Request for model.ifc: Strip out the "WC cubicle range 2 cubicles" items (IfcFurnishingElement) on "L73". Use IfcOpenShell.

First a look at what the model holds.

```python
import ifcopenshell
import ifcopenshell.util.element

model = ifcopenshell.open("model.ifc")
print(model.schema)
storey = next(s for s in model.by_type("IfcBuildingStorey") if s.Name == "L73")
furniture = [e for e in ifcopenshell.util.element.get_decomposition(storey) if e.is_a("IfcFurnishingElement")]
seen = {}
for e in furniture:
    element_type = ifcopenshell.util.element.get_type(e)
    name = element_type.Name if element_type not in (None, e) else None
    seen[name] = seen.get(name, 0) + 1
for name, count in sorted(seen.items(), key=str):
    print(count, "x", name)
```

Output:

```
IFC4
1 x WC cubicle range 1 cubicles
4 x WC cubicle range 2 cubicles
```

```python
import ifcopenshell
import ifcopenshell.api.root
import ifcopenshell.util.element

model = ifcopenshell.open("model.ifc")

storey = next(s for s in model.by_type("IfcBuildingStorey") if s.Name == "L73")
furniture = [e for e in ifcopenshell.util.element.get_decomposition(storey) if e.is_a("IfcFurnishingElement")]
targets = [e for e in furniture if (t := ifcopenshell.util.element.get_type(e)) not in (None, e) and t.Name == "WC cubicle range 2 cubicles"]

for e in targets:
    ifcopenshell.api.root.remove_product(model, product=e)
print(len(targets), "removed")

model.write("model_rev.ifc")
```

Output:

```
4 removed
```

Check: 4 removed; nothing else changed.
